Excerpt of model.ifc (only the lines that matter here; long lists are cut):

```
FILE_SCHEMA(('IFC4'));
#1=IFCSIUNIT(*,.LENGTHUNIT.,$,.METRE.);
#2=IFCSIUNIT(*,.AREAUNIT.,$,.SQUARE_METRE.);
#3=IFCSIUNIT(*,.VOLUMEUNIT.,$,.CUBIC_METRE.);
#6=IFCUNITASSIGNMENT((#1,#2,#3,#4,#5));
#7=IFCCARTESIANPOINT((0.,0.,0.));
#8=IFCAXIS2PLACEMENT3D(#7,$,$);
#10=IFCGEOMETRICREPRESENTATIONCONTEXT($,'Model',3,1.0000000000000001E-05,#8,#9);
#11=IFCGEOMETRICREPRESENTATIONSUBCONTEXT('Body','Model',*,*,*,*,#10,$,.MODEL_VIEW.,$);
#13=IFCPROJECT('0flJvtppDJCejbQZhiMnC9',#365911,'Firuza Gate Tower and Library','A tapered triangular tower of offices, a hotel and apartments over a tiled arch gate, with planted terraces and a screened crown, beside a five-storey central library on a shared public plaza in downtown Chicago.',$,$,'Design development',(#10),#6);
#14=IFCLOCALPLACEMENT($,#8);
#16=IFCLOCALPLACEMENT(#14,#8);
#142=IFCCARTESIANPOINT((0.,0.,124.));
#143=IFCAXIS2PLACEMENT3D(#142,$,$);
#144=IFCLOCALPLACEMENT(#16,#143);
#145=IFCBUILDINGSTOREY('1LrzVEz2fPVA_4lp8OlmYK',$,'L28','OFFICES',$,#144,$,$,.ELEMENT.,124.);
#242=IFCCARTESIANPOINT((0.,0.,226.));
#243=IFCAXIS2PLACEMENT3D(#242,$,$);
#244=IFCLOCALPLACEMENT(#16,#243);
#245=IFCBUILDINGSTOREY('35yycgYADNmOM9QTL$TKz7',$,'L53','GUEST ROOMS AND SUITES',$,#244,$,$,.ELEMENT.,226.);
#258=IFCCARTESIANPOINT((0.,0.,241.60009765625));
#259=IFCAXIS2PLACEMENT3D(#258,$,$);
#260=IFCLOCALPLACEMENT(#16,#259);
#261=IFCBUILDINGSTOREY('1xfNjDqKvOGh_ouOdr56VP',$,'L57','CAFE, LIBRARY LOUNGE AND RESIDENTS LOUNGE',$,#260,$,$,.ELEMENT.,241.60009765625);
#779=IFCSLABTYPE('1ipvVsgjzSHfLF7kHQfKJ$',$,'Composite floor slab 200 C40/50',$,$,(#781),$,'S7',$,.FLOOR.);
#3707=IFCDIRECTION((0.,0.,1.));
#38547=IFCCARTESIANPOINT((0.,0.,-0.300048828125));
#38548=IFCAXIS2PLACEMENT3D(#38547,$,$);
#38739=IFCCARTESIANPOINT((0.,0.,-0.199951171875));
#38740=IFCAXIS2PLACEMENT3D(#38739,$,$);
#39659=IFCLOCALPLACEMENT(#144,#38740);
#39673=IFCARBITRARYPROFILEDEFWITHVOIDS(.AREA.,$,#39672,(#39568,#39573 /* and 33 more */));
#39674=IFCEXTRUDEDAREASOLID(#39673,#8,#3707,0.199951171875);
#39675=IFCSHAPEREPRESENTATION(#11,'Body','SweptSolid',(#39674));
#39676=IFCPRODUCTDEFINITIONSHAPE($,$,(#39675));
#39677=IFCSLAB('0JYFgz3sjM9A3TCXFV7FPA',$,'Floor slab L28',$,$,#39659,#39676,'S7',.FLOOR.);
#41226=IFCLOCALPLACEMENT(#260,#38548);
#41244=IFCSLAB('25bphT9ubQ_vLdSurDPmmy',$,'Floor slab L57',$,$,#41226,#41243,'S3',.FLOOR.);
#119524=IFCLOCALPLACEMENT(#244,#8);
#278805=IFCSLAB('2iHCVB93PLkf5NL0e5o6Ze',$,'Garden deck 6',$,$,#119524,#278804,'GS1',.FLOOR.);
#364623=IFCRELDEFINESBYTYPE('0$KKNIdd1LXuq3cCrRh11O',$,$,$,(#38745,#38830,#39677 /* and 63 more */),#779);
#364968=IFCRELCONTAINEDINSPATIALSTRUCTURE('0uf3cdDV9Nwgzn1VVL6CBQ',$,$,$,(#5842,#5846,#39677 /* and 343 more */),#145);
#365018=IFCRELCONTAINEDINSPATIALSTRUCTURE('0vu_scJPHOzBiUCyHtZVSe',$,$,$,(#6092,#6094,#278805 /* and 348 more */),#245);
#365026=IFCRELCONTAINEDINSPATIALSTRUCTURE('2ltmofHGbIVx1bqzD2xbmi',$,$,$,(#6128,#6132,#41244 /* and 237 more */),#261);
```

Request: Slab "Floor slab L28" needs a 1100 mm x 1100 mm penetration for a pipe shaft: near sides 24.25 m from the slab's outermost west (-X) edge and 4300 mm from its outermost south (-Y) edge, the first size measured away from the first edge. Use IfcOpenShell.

```python
import numpy as np
import ifcopenshell
import ifcopenshell.api.feature
import ifcopenshell.api.geometry
import ifcopenshell.api.root
import ifcopenshell.geom
import ifcopenshell.util.placement
import ifcopenshell.util.representation
import ifcopenshell.util.shape
import ifcopenshell.util.unit

model = ifcopenshell.open("model.ifc")
unit_scale = ifcopenshell.util.unit.calculate_unit_scale(model)
settings = ifcopenshell.geom.settings()


def volume(element):
    """Net volume in cubic metres, openings subtracted."""
    shape = ifcopenshell.geom.create_shape(settings, element)
    return ifcopenshell.util.shape.get_volume(shape.geometry)


slab = model.by_guid("0JYFgz3sjM9A3TCXFV7FPA")
before = volume(slab)

# Extent in the slab's own axes, in metres. The edges named are its -X and -Y sides.
slab_shape = ifcopenshell.geom.create_shape(settings, slab)
vertices = ifcopenshell.util.shape.get_vertices(slab_shape.geometry)
x_min, y_min, bottom = vertices.min(axis=0)
top = vertices[:, 2].max()

opening = ifcopenshell.api.root.create_entity(model, ifc_class="IfcOpeningElement", name="Pipe shaft opening", predefined_type="OPENING")
context = ifcopenshell.util.representation.get_context(model, "Model", "Body", "MODEL_VIEW")
width, depth = 1.1, 1.1
outline = [(0.0, 0.0), (width, 0.0), (width, depth), (0.0, depth), (0.0, 0.0)]
# Overshoot both faces by 50 mm so the cut is clean.
shape = ifcopenshell.api.geometry.add_slab_representation(
    model, context=context, depth=top - bottom + 0.1, polyline=outline
)
ifcopenshell.api.geometry.assign_representation(model, product=opening, representation=shape)

matrix = ifcopenshell.util.placement.get_local_placement(slab.ObjectPlacement)
matrix[:, 3] = matrix @ np.append(np.array([x_min + 24.25, y_min + 4.3, bottom - 0.05]) / unit_scale, 1.0)
ifcopenshell.api.geometry.edit_object_placement(model, product=opening, matrix=matrix, is_si=False)
ifcopenshell.api.feature.add_feature(model, feature=opening, element=slab)

after = volume(slab)

print(f"slab volume {before:.3f} -> {after:.3f} m3")

model.write("model_rev.ifc")
```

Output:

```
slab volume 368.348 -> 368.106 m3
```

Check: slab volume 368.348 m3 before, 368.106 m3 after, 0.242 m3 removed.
